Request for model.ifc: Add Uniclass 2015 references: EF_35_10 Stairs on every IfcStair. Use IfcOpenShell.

First a look at what the model holds.

```python
import ifcopenshell

model = ifcopenshell.open("model.ifc")
print(model.schema)
print("classifications:", [c.Name for c in model.by_type("IfcClassification")])
for ifc_class in ("IfcDoor", "IfcRoof", "IfcStair", "IfcWall", "IfcWindow"):
    print(ifc_class, len(model.by_type(ifc_class)))
```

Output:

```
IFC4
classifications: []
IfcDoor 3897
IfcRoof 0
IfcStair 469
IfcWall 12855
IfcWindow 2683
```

```python
import ifcopenshell
import ifcopenshell.api.classification

model = ifcopenshell.open("model.ifc")

system = ifcopenshell.api.classification.add_classification(model, classification="Uniclass 2015")

codes = {
    "IfcStair": ("EF_35_10", "Stairs"),
}
for ifc_class, (code, name) in codes.items():
    products = model.by_type(ifc_class)
    ifcopenshell.api.classification.add_reference(
        model, products=products, classification=system, identification=code, name=name
    )
    print(code, len(products))

model.write("model_v2.ifc")
```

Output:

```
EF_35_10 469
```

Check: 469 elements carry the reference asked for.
